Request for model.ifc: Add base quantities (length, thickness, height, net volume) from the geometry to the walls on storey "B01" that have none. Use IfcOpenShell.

First a look at what the model holds.

```python
import ifcopenshell
import ifcopenshell.util.element
import ifcopenshell.util.unit

model = ifcopenshell.open("model.ifc")
print(model.schema)
for unit_type in ("LENGTHUNIT", "AREAUNIT", "VOLUMEUNIT"):
    print(unit_type, ifcopenshell.util.unit.calculate_unit_scale(model, unit_type))
storey = next(s for s in model.by_type("IfcBuildingStorey") if s.Name == "B01")
walls = [e for e in ifcopenshell.util.element.get_decomposition(storey) if e.is_a("IfcWall")]
for e in sorted(walls, key=lambda e: e.id()):
    print(e.id(), e.is_a(), e.Name, list(ifcopenshell.util.element.get_psets(e, qtos_only=True)), sep=" | ")
```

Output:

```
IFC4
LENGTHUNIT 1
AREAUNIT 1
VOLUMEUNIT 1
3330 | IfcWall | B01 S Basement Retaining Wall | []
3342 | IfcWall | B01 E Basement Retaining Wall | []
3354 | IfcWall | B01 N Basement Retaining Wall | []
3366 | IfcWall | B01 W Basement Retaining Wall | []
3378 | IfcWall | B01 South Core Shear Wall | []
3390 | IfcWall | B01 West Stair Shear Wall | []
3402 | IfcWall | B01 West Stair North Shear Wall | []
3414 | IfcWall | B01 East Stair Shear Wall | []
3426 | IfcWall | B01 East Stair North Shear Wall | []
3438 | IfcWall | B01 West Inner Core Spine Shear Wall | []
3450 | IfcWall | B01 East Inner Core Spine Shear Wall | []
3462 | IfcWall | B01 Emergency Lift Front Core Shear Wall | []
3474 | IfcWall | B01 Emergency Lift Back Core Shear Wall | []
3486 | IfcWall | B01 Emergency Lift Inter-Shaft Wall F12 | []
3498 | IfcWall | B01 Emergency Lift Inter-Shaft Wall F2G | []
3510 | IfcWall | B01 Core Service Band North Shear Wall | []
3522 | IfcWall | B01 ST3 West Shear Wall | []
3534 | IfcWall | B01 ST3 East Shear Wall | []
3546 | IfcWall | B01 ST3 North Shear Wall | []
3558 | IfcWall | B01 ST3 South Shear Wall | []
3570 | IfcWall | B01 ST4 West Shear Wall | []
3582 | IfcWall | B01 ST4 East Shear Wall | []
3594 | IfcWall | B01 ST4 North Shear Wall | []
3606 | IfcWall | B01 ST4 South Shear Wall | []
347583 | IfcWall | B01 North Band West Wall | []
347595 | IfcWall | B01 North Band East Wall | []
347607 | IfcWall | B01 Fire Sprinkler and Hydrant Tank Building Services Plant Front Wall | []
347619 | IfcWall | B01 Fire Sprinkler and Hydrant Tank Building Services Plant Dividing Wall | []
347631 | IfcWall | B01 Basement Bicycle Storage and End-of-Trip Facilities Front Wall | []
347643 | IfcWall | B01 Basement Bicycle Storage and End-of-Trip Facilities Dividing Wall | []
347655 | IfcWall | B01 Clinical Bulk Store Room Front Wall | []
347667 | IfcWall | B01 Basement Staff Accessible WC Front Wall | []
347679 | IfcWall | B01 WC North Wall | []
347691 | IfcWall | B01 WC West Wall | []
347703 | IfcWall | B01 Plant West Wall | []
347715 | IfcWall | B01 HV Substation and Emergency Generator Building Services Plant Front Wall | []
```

```python
import ifcopenshell
import ifcopenshell.api.pset
import ifcopenshell.geom
import ifcopenshell.util.element
import ifcopenshell.util.shape
import ifcopenshell.util.unit

model = ifcopenshell.open("model.ifc")
unit_scale = ifcopenshell.util.unit.calculate_unit_scale(model)
volume_scale = ifcopenshell.util.unit.calculate_unit_scale(model, "VOLUMEUNIT")
settings = ifcopenshell.geom.settings()

storey = next(s for s in model.by_type("IfcBuildingStorey") if s.Name == "B01")
walls = [e for e in ifcopenshell.util.element.get_decomposition(storey) if e.is_a("IfcWall")]

for e in sorted(walls, key=lambda e: e.id()):
    if ifcopenshell.util.element.get_psets(e, qtos_only=True, should_inherit=False):
        continue
    # Geometry comes back in metres, in the element's own axes.
    shape = ifcopenshell.geom.create_shape(settings, e)
    values = {
        "Length": ifcopenshell.util.shape.get_x(shape.geometry) / unit_scale,
        "Width": ifcopenshell.util.shape.get_y(shape.geometry) / unit_scale,
        "Height": ifcopenshell.util.shape.get_z(shape.geometry) / unit_scale,
        "NetVolume": ifcopenshell.util.shape.get_volume(shape.geometry) / volume_scale,
    }
    qto = ifcopenshell.api.pset.add_qto(model, product=e, name="Qto_WallBaseQuantities")
    ifcopenshell.api.pset.edit_qto(model, qto=qto, properties=values)
    print(e.id(), {k: round(v, 3) for k, v in values.items()})

model.write("model_v2.ifc")
```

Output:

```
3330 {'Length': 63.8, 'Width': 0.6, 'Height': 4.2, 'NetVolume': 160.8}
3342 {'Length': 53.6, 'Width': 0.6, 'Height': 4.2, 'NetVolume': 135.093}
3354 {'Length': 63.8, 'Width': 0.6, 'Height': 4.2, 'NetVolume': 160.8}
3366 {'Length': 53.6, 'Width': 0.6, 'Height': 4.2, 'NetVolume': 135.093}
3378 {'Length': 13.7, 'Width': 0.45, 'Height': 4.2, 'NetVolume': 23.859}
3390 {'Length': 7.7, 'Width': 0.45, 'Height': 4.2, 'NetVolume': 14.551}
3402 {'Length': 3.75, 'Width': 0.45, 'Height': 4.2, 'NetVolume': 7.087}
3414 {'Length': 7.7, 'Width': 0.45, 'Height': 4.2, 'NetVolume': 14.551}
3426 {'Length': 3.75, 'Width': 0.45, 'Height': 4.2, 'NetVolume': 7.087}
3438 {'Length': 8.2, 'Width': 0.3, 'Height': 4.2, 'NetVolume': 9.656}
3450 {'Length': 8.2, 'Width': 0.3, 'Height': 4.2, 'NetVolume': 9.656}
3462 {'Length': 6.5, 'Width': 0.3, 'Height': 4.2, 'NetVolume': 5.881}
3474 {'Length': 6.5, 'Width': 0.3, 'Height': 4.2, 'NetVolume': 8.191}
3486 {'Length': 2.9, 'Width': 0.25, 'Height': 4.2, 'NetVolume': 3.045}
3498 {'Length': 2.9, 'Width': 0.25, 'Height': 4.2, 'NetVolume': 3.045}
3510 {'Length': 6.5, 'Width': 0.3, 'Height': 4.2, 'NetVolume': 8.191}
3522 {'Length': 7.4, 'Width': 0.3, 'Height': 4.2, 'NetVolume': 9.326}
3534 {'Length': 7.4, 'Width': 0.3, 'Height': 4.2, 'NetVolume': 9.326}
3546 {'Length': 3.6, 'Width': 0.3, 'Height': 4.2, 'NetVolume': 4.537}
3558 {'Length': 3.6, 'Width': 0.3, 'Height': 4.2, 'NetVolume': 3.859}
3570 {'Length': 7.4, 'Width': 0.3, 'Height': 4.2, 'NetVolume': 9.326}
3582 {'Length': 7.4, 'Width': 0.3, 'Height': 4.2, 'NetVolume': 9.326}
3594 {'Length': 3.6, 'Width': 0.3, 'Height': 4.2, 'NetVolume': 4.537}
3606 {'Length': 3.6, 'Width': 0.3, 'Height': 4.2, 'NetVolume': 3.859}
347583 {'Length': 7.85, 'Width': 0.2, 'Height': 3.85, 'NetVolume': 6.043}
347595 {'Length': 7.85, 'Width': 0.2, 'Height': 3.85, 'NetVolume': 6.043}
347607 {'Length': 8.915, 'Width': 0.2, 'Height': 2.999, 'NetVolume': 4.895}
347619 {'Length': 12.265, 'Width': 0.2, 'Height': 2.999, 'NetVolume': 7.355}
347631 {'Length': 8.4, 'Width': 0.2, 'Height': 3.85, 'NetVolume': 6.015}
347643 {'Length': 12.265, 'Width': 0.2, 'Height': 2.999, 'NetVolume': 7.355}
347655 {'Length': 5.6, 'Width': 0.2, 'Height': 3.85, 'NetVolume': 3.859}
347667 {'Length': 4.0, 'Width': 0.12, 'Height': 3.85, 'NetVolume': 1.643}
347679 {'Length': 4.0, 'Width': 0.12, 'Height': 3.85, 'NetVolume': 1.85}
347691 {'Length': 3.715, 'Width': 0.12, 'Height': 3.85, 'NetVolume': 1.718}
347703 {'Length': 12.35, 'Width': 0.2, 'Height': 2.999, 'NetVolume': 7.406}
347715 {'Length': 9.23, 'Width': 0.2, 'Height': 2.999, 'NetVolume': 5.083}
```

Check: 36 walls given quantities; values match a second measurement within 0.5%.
